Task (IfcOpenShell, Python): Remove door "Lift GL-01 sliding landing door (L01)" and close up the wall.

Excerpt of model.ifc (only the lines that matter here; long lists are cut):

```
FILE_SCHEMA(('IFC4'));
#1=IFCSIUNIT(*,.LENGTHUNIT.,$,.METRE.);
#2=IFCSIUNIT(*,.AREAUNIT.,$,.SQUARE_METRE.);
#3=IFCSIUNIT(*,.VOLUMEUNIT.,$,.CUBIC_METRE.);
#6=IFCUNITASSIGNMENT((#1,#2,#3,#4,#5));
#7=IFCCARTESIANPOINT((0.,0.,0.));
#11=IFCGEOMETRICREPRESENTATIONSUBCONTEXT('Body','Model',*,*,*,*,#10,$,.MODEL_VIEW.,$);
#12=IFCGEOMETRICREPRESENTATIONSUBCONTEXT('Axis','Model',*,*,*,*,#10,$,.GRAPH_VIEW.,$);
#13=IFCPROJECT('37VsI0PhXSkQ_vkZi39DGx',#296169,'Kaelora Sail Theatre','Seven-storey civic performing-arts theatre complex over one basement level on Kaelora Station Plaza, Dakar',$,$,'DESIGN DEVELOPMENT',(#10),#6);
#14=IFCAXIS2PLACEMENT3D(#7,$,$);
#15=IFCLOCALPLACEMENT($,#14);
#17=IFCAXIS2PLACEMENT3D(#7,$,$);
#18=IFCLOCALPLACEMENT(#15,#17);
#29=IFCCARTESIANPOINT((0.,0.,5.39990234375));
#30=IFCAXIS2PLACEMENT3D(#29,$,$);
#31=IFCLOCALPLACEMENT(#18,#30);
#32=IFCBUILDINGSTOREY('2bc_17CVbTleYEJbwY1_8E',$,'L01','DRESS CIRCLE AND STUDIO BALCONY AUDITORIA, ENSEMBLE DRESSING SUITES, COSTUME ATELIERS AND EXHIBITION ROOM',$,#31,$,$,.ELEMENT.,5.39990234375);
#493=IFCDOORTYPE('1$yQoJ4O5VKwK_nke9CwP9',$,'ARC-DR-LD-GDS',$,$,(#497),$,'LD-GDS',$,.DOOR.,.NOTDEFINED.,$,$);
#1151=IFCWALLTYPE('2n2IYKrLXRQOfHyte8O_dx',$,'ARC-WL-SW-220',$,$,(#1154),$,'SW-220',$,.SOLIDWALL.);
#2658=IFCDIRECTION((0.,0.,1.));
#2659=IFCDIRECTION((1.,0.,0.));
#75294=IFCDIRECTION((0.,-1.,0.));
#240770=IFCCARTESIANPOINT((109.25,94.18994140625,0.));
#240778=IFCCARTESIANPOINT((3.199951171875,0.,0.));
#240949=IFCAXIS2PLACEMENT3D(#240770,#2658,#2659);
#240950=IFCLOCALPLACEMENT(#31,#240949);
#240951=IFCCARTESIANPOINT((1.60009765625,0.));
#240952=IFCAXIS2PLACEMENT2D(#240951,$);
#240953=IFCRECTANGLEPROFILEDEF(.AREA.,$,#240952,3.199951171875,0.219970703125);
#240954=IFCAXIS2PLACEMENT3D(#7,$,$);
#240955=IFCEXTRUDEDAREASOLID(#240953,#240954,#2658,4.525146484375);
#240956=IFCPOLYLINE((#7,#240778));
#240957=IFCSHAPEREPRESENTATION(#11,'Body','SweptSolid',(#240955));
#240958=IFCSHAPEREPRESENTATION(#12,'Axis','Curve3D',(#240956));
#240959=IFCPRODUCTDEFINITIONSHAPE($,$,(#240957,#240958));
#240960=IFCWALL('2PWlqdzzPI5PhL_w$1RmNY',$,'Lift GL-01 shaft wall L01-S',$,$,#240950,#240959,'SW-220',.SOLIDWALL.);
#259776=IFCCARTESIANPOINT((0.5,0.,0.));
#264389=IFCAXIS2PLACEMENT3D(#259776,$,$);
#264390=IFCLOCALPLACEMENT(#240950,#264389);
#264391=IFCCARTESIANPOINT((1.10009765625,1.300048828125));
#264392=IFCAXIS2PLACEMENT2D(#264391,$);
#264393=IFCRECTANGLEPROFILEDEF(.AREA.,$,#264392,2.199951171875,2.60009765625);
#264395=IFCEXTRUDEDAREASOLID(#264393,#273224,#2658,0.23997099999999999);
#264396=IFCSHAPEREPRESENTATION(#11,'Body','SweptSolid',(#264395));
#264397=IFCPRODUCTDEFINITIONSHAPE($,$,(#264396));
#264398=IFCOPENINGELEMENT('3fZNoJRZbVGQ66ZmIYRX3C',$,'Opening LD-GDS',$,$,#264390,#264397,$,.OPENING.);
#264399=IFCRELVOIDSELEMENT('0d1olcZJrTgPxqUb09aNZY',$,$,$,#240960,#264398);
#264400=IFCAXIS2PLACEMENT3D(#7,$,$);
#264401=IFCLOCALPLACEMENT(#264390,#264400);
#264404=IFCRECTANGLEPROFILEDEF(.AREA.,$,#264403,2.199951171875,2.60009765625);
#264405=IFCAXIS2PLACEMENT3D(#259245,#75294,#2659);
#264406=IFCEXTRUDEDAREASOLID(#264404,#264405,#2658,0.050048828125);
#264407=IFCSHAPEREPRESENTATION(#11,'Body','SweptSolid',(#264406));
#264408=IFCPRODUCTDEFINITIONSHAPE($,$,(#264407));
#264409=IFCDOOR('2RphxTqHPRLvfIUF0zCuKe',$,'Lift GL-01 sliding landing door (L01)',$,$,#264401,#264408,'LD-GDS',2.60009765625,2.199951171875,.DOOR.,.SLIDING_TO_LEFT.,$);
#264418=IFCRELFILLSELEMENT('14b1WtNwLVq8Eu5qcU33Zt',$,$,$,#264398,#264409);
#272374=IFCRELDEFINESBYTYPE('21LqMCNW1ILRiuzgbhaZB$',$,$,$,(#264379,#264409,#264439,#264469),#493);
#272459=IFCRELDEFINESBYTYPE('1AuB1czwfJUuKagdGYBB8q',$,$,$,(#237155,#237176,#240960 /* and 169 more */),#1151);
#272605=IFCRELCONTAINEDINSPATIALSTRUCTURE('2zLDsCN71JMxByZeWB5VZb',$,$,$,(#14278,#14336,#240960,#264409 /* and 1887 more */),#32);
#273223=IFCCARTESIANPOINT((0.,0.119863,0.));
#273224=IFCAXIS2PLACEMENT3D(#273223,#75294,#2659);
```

```python
import ifcopenshell
import ifcopenshell.api.feature
import ifcopenshell.api.root
import ifcopenshell.geom
import ifcopenshell.util.shape

model = ifcopenshell.open("model.ifc")
settings = ifcopenshell.geom.settings()


def volume(element):
    """Net volume in cubic metres, openings subtracted."""
    shape = ifcopenshell.geom.create_shape(settings, element)
    return ifcopenshell.util.shape.get_volume(shape.geometry)


door = model.by_guid("2RphxTqHPRLvfIUF0zCuKe")
opening = door.FillsVoids[0].RelatingOpeningElement
wall = opening.VoidsElements[0].RelatingBuildingElement
before = volume(wall)

ifcopenshell.api.root.remove_product(model, product=door)
ifcopenshell.api.feature.remove_feature(model, feature=opening)

after = volume(wall)

print(f"wall volume {before:.3f} -> {after:.3f} m3")

model.write("model_rev.ifc")
```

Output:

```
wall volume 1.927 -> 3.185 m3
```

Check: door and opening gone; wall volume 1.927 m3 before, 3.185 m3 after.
